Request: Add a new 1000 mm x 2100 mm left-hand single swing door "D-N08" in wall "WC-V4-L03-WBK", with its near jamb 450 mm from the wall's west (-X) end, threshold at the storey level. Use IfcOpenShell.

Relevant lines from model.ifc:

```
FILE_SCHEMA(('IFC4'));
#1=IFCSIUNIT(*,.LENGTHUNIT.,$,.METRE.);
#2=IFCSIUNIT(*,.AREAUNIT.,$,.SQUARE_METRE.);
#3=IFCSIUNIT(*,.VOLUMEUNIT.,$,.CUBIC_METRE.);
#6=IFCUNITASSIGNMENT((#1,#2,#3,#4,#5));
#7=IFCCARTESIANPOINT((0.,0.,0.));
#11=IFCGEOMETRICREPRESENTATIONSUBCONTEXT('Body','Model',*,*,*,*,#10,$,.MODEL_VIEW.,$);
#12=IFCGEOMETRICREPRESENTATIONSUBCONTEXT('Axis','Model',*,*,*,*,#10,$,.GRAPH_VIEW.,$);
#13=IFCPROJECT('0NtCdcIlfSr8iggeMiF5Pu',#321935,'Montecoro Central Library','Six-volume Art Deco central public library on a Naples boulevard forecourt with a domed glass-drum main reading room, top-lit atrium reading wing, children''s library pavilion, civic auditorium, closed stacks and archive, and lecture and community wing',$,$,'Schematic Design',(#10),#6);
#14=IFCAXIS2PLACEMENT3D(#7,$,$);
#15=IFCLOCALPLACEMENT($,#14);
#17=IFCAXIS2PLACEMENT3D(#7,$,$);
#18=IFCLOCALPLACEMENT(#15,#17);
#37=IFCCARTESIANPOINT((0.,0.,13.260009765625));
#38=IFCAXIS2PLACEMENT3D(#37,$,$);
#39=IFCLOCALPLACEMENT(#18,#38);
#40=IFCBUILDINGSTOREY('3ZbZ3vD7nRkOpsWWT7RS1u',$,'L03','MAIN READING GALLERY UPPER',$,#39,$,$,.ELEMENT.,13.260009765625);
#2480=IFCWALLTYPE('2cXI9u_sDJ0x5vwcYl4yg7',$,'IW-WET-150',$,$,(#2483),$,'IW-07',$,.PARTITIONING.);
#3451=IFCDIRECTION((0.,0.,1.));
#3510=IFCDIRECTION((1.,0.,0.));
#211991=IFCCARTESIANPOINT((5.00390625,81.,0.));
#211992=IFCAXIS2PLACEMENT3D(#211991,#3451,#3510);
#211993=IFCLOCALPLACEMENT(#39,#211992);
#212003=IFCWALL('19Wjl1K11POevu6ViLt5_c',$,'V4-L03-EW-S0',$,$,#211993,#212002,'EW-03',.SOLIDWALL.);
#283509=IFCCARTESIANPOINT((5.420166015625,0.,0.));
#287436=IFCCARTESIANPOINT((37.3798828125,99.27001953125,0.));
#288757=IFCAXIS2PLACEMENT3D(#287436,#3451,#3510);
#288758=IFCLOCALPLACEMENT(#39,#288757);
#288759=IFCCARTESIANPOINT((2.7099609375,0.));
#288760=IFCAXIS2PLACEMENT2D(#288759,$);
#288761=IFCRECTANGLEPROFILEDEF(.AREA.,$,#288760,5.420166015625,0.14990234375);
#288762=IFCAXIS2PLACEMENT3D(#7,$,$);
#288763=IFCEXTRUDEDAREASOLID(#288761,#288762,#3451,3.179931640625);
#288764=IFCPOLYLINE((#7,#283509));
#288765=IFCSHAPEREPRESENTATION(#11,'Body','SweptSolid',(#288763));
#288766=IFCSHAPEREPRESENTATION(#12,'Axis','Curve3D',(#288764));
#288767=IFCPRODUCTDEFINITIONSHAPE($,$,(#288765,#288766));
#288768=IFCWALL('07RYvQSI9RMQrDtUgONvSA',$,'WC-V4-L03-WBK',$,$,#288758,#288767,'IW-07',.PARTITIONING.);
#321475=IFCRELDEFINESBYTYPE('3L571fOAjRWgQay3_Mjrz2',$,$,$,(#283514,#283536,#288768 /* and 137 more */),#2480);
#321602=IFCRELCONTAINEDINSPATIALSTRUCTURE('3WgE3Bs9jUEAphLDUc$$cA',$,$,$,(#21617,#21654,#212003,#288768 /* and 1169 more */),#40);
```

```python
import numpy as np
import ifcopenshell
import ifcopenshell.api.feature
import ifcopenshell.api.geometry
import ifcopenshell.api.root
import ifcopenshell.api.spatial
import ifcopenshell.geom
import ifcopenshell.util.element
import ifcopenshell.util.placement
import ifcopenshell.util.representation
import ifcopenshell.util.shape
import ifcopenshell.util.unit

model = ifcopenshell.open("model.ifc")
unit_scale = ifcopenshell.util.unit.calculate_unit_scale(model)
settings = ifcopenshell.geom.settings()


def volume(element):
    """Net volume in cubic metres, openings subtracted."""
    shape = ifcopenshell.geom.create_shape(settings, element)
    return ifcopenshell.util.shape.get_volume(shape.geometry)


wall = model.by_guid("07RYvQSI9RMQrDtUgONvSA")
storey = ifcopenshell.util.element.get_container(wall, ifc_class="IfcBuildingStorey")
context = ifcopenshell.util.representation.get_context(model, "Model", "Body", "MODEL_VIEW")
before = volume(wall)

width, height, from_end, sill = 1, 2.1, 0.45, 0.0  # metres

# The wall runs along its own X axis, and the end named is its -X end.
wall_shape = ifcopenshell.geom.create_shape(settings, wall)
x, y, z = ifcopenshell.util.shape.get_vertices(wall_shape.geometry).T
start = x.min() + from_end
face, thickness = float(y.min()), float(y.max() - y.min())
wall_matrix = ifcopenshell.util.placement.get_local_placement(wall.ObjectPlacement)
level = ifcopenshell.util.placement.get_local_placement(storey.ObjectPlacement)[2, 3]


def in_wall(x, y):
    """Placement at x, y metres in the wall's axes, at sill height."""
    matrix = wall_matrix.copy()
    matrix[:, 3] = wall_matrix @ np.array([x / unit_scale, y / unit_scale, 0.0, 1.0])
    matrix[2, 3] = level + sill / unit_scale
    return matrix


# Opening: a box that overshoots both wall faces by 50 mm.
opening = ifcopenshell.api.root.create_entity(model, ifc_class="IfcOpeningElement", predefined_type="OPENING")
box = ifcopenshell.api.geometry.add_wall_representation(
    model, context=context, length=width, height=height, thickness=thickness + 0.1
)
ifcopenshell.api.geometry.assign_representation(model, product=opening, representation=box)
ifcopenshell.api.geometry.edit_object_placement(model, product=opening, matrix=in_wall(start, face - 0.05), is_si=False)
ifcopenshell.api.feature.add_feature(model, feature=opening, element=wall)

door = ifcopenshell.api.root.create_entity(model, ifc_class="IfcDoor", name="D-N08", predefined_type="DOOR")
door.OverallWidth, door.OverallHeight = width / unit_scale, height / unit_scale
door.OperationType = "SINGLE_SWING_LEFT"
body = ifcopenshell.api.geometry.add_door_representation(
    model,
    context=context,
    overall_width=door.OverallWidth,
    overall_height=door.OverallHeight,
    operation_type="SINGLE_SWING_LEFT",
    lining_properties={"LiningDepth": thickness / unit_scale, "ThresholdDepth": thickness / unit_scale},
)
ifcopenshell.api.geometry.assign_representation(model, product=door, representation=body)
ifcopenshell.api.spatial.assign_container(model, products=[door], relating_structure=storey)
ifcopenshell.api.feature.add_filling(model, opening=opening, element=door)

# The lining spans the wall, so the door starts at the wall face.
ifcopenshell.api.geometry.edit_object_placement(model, product=door, matrix=in_wall(start, face), is_si=False)

after = volume(wall)

print(f"wall volume {before:.3f} -> {after:.3f} m3")

model.write("model_updated.ifc")
```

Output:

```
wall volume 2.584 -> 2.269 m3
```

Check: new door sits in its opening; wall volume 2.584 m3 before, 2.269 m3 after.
